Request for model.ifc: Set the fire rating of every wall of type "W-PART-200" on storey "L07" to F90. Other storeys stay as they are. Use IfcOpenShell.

First a look at what the model holds.

```python
import ifcopenshell
import ifcopenshell.util.element

model = ifcopenshell.open("model.ifc")
print(model.schema)
storey = next(s for s in model.by_type("IfcBuildingStorey") if s.Name == "L07")
walls = [e for e in ifcopenshell.util.element.get_decomposition(storey) if e.is_a("IfcWall")]
seen = {}
for e in walls:
    element_type = ifcopenshell.util.element.get_type(e)
    key = (element_type.Name if element_type != e and element_type else None, ifcopenshell.util.element.get_pset(e, "Pset_WallCommon", "FireRating"))
    seen[key] = seen.get(key, 0) + 1
for (name, value), count in sorted(seen.items(), key=str):
    print(count, "x", name, "|", value)
```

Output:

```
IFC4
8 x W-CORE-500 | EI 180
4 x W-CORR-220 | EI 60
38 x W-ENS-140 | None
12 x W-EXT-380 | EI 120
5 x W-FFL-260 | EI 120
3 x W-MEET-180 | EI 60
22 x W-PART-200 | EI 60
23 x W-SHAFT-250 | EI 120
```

```python
import ifcopenshell
import ifcopenshell.api.pset
import ifcopenshell.util.element

model = ifcopenshell.open("model.ifc")

storey = next(s for s in model.by_type("IfcBuildingStorey") if s.Name == "L07")
walls = [e for e in ifcopenshell.util.element.get_decomposition(storey) if e.is_a("IfcWall")]

count = 0
for e in walls:
    element_type = ifcopenshell.util.element.get_type(e)
    if element_type in (None, e) or element_type.Name != "W-PART-200":
        continue
    # add_pset returns the element's existing set when there is one.
    pset = ifcopenshell.api.pset.add_pset(model, product=e, name="Pset_WallCommon")
    ifcopenshell.api.pset.edit_pset(model, pset=pset, properties={"FireRating": "F90"})
    count += 1

print(count, "walls updated")

model.write("model_edited.ifc")
```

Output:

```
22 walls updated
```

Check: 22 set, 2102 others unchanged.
